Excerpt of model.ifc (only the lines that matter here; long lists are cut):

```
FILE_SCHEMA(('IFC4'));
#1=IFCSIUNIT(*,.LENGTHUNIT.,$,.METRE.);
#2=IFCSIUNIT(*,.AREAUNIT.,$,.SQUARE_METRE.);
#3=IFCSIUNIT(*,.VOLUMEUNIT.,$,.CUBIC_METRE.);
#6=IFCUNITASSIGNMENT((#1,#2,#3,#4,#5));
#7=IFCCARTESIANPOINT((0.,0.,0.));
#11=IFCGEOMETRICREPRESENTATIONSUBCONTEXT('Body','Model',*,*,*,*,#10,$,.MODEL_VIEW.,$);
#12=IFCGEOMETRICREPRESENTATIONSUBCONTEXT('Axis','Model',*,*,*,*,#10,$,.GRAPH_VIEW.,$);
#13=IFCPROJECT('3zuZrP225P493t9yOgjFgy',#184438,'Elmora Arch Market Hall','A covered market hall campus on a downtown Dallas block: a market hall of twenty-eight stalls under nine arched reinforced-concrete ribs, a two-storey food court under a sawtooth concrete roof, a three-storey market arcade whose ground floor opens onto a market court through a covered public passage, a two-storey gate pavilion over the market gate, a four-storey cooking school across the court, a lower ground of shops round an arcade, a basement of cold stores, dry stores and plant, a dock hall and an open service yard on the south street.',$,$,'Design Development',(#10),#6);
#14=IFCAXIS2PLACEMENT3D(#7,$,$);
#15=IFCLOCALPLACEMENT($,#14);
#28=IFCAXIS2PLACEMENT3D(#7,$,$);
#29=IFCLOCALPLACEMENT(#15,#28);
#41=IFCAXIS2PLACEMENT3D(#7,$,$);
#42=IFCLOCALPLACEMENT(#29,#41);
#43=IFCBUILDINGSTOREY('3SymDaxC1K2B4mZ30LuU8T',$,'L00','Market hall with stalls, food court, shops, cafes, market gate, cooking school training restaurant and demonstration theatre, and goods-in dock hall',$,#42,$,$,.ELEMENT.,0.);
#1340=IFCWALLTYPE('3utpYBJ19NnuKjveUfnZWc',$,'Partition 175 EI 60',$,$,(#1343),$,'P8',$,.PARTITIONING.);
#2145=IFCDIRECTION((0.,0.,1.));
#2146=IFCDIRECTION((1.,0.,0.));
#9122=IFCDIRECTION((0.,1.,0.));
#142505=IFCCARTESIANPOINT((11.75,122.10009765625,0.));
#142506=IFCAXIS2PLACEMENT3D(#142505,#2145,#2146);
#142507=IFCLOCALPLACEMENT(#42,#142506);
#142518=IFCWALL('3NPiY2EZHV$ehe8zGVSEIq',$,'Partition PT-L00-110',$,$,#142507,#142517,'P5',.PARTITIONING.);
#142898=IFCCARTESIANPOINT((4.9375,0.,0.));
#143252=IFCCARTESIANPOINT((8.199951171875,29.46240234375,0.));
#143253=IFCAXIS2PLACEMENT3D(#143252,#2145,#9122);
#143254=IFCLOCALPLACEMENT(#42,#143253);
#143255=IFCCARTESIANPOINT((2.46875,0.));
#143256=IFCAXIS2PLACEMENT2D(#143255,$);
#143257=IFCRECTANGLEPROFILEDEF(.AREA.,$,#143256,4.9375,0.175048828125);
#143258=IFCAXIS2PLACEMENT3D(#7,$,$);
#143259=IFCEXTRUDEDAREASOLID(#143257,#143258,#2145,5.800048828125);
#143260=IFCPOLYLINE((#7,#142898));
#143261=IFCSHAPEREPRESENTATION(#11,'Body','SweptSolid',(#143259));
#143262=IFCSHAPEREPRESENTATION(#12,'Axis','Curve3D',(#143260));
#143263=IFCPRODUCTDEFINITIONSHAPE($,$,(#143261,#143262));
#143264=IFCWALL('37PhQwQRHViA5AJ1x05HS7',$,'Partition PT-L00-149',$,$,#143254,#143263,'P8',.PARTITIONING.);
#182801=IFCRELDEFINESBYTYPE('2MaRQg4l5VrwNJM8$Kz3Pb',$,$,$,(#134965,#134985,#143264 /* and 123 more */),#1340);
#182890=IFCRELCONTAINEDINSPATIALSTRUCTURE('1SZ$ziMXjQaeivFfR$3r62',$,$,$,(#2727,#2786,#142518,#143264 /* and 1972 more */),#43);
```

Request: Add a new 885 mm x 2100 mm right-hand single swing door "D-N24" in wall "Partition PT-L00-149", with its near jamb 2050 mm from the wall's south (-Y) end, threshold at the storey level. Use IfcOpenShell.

```python
import numpy as np
import ifcopenshell
import ifcopenshell.api.feature
import ifcopenshell.api.geometry
import ifcopenshell.api.root
import ifcopenshell.api.spatial
import ifcopenshell.geom
import ifcopenshell.util.element
import ifcopenshell.util.placement
import ifcopenshell.util.representation
import ifcopenshell.util.shape
import ifcopenshell.util.unit

model = ifcopenshell.open("model.ifc")
unit_scale = ifcopenshell.util.unit.calculate_unit_scale(model)
settings = ifcopenshell.geom.settings()


def volume(element):
    """Net volume in cubic metres, openings subtracted."""
    shape = ifcopenshell.geom.create_shape(settings, element)
    return ifcopenshell.util.shape.get_volume(shape.geometry)


wall = model.by_guid("37PhQwQRHViA5AJ1x05HS7")
storey = ifcopenshell.util.element.get_container(wall, ifc_class="IfcBuildingStorey")
context = ifcopenshell.util.representation.get_context(model, "Model", "Body", "MODEL_VIEW")
before = volume(wall)

width, height, from_end, sill = 0.885, 2.1, 2.05, 0.0  # metres

# The wall runs along its own X axis, and the end named is its -X end.
wall_shape = ifcopenshell.geom.create_shape(settings, wall)
x, y, z = ifcopenshell.util.shape.get_vertices(wall_shape.geometry).T
start = x.min() + from_end
face, thickness = float(y.min()), float(y.max() - y.min())
wall_matrix = ifcopenshell.util.placement.get_local_placement(wall.ObjectPlacement)
level = ifcopenshell.util.placement.get_local_placement(storey.ObjectPlacement)[2, 3]


def in_wall(x, y):
    """Placement at x, y metres in the wall's axes, at sill height."""
    matrix = wall_matrix.copy()
    matrix[:, 3] = wall_matrix @ np.array([x / unit_scale, y / unit_scale, 0.0, 1.0])
    matrix[2, 3] = level + sill / unit_scale
    return matrix


# Opening: a box that overshoots both wall faces by 50 mm.
opening = ifcopenshell.api.root.create_entity(model, ifc_class="IfcOpeningElement", predefined_type="OPENING")
box = ifcopenshell.api.geometry.add_wall_representation(
    model, context=context, length=width, height=height, thickness=thickness + 0.1
)
ifcopenshell.api.geometry.assign_representation(model, product=opening, representation=box)
ifcopenshell.api.geometry.edit_object_placement(model, product=opening, matrix=in_wall(start, face - 0.05), is_si=False)
ifcopenshell.api.feature.add_feature(model, feature=opening, element=wall)

door = ifcopenshell.api.root.create_entity(model, ifc_class="IfcDoor", name="D-N24", predefined_type="DOOR")
door.OverallWidth, door.OverallHeight = width / unit_scale, height / unit_scale
door.OperationType = "SINGLE_SWING_RIGHT"
body = ifcopenshell.api.geometry.add_door_representation(
    model,
    context=context,
    overall_width=door.OverallWidth,
    overall_height=door.OverallHeight,
    operation_type="SINGLE_SWING_RIGHT",
    lining_properties={"LiningDepth": thickness / unit_scale, "ThresholdDepth": thickness / unit_scale},
)
ifcopenshell.api.geometry.assign_representation(model, product=door, representation=body)
ifcopenshell.api.spatial.assign_container(model, products=[door], relating_structure=storey)
ifcopenshell.api.feature.add_filling(model, opening=opening, element=door)

# The lining spans the wall, so the door starts at the wall face.
ifcopenshell.api.geometry.edit_object_placement(model, product=door, matrix=in_wall(start, face), is_si=False)

after = volume(wall)

print(f"wall volume {before:.3f} -> {after:.3f} m3")

model.write("model_v2.ifc")
```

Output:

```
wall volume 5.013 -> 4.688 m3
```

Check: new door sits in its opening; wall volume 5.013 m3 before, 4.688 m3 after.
